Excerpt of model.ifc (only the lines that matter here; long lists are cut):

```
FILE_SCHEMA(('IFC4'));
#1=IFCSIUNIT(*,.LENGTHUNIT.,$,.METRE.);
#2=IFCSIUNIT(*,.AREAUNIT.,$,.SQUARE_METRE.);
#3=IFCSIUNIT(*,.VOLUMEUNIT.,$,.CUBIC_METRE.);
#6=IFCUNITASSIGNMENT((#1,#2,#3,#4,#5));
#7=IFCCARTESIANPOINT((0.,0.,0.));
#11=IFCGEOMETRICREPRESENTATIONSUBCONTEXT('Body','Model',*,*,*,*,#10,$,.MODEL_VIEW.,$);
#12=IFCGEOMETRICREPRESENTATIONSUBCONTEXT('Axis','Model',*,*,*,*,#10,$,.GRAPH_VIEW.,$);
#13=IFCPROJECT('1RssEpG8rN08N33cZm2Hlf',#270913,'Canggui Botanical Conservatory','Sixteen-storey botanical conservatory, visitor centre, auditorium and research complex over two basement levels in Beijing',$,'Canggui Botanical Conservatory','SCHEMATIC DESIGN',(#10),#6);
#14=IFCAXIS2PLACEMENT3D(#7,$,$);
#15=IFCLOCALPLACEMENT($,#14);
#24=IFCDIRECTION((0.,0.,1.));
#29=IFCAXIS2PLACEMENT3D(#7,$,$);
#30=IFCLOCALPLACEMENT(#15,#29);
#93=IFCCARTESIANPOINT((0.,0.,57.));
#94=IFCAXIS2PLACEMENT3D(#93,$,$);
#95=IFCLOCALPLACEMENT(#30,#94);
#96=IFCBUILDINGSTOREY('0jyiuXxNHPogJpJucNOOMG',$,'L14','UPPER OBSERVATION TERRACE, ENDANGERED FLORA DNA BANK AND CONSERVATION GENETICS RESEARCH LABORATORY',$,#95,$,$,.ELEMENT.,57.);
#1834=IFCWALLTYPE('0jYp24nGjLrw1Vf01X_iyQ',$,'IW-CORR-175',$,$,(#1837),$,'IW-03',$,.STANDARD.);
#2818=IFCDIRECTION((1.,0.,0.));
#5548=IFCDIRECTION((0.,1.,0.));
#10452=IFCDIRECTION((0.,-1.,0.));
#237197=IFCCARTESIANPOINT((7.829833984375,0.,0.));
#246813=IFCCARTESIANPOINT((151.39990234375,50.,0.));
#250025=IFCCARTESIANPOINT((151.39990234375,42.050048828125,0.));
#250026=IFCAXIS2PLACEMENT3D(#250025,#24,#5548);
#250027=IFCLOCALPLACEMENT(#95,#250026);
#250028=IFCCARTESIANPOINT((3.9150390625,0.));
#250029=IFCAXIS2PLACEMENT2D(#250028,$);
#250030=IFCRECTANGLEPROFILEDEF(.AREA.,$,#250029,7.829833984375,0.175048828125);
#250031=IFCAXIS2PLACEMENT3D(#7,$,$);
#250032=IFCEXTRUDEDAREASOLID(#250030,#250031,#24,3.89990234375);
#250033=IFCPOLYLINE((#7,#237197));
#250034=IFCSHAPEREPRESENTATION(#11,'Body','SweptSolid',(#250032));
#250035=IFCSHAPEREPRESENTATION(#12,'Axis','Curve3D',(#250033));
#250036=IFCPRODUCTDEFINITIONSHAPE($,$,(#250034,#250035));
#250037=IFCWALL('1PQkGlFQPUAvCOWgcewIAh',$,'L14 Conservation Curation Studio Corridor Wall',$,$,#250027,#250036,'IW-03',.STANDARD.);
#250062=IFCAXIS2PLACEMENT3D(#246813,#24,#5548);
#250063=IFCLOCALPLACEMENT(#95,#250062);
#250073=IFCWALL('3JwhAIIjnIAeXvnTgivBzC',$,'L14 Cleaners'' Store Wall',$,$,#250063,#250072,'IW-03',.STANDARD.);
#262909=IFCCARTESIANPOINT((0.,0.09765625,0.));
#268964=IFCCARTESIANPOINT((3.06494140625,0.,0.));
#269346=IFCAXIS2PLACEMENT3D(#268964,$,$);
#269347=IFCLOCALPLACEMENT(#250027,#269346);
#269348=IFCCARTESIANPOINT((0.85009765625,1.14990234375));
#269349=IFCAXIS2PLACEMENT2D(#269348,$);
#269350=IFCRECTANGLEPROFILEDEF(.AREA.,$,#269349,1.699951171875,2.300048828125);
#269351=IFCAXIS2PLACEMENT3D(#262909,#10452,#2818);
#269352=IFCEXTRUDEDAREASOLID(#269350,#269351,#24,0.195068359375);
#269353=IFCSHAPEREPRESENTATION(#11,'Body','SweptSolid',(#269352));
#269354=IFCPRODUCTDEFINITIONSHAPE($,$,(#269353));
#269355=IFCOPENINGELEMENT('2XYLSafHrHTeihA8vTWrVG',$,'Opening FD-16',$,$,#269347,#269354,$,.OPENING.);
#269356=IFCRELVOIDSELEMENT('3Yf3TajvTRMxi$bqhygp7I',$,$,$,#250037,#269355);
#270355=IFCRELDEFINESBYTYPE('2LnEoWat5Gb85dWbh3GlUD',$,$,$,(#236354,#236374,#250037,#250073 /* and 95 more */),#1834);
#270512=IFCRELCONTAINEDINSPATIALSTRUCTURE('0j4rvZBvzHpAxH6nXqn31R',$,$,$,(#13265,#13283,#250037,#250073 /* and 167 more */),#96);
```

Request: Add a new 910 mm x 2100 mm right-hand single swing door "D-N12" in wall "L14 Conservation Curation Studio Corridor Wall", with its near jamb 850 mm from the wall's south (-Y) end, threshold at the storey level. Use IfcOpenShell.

```python
import numpy as np
import ifcopenshell
import ifcopenshell.api.feature
import ifcopenshell.api.geometry
import ifcopenshell.api.root
import ifcopenshell.api.spatial
import ifcopenshell.geom
import ifcopenshell.util.element
import ifcopenshell.util.placement
import ifcopenshell.util.representation
import ifcopenshell.util.shape
import ifcopenshell.util.unit

model = ifcopenshell.open("model.ifc")
unit_scale = ifcopenshell.util.unit.calculate_unit_scale(model)
settings = ifcopenshell.geom.settings()


def volume(element):
    """Net volume in cubic metres, openings subtracted."""
    shape = ifcopenshell.geom.create_shape(settings, element)
    return ifcopenshell.util.shape.get_volume(shape.geometry)


wall = model.by_guid("1PQkGlFQPUAvCOWgcewIAh")
storey = ifcopenshell.util.element.get_container(wall, ifc_class="IfcBuildingStorey")
context = ifcopenshell.util.representation.get_context(model, "Model", "Body", "MODEL_VIEW")
before = volume(wall)

width, height, from_end, sill = 0.91, 2.1, 0.85, 0.0  # metres

# The wall runs along its own X axis, and the end named is its -X end.
wall_shape = ifcopenshell.geom.create_shape(settings, wall)
x, y, z = ifcopenshell.util.shape.get_vertices(wall_shape.geometry).T
start = x.min() + from_end
face, thickness = float(y.min()), float(y.max() - y.min())
wall_matrix = ifcopenshell.util.placement.get_local_placement(wall.ObjectPlacement)
level = ifcopenshell.util.placement.get_local_placement(storey.ObjectPlacement)[2, 3]


def in_wall(x, y):
    """Placement at x, y metres in the wall's axes, at sill height."""
    matrix = wall_matrix.copy()
    matrix[:, 3] = wall_matrix @ np.array([x / unit_scale, y / unit_scale, 0.0, 1.0])
    matrix[2, 3] = level + sill / unit_scale
    return matrix


# Opening: a box that overshoots both wall faces by 50 mm.
opening = ifcopenshell.api.root.create_entity(model, ifc_class="IfcOpeningElement", predefined_type="OPENING")
box = ifcopenshell.api.geometry.add_wall_representation(
    model, context=context, length=width, height=height, thickness=thickness + 0.1
)
ifcopenshell.api.geometry.assign_representation(model, product=opening, representation=box)
ifcopenshell.api.geometry.edit_object_placement(model, product=opening, matrix=in_wall(start, face - 0.05), is_si=False)
ifcopenshell.api.feature.add_feature(model, feature=opening, element=wall)

door = ifcopenshell.api.root.create_entity(model, ifc_class="IfcDoor", name="D-N12", predefined_type="DOOR")
door.OverallWidth, door.OverallHeight = width / unit_scale, height / unit_scale
door.OperationType = "SINGLE_SWING_RIGHT"
body = ifcopenshell.api.geometry.add_door_representation(
    model,
    context=context,
    overall_width=door.OverallWidth,
    overall_height=door.OverallHeight,
    operation_type="SINGLE_SWING_RIGHT",
    lining_properties={"LiningDepth": thickness / unit_scale, "ThresholdDepth": thickness / unit_scale},
)
ifcopenshell.api.geometry.assign_representation(model, product=door, representation=body)
ifcopenshell.api.spatial.assign_container(model, products=[door], relating_structure=storey)
ifcopenshell.api.feature.add_filling(model, opening=opening, element=door)

# The lining spans the wall, so the door starts at the wall face.
ifcopenshell.api.geometry.edit_object_placement(model, product=door, matrix=in_wall(start, face), is_si=False)

after = volume(wall)

print(f"wall volume {before:.3f} -> {after:.3f} m3")

model.write("model_rev.ifc")
```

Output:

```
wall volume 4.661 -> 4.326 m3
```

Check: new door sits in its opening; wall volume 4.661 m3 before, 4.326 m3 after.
